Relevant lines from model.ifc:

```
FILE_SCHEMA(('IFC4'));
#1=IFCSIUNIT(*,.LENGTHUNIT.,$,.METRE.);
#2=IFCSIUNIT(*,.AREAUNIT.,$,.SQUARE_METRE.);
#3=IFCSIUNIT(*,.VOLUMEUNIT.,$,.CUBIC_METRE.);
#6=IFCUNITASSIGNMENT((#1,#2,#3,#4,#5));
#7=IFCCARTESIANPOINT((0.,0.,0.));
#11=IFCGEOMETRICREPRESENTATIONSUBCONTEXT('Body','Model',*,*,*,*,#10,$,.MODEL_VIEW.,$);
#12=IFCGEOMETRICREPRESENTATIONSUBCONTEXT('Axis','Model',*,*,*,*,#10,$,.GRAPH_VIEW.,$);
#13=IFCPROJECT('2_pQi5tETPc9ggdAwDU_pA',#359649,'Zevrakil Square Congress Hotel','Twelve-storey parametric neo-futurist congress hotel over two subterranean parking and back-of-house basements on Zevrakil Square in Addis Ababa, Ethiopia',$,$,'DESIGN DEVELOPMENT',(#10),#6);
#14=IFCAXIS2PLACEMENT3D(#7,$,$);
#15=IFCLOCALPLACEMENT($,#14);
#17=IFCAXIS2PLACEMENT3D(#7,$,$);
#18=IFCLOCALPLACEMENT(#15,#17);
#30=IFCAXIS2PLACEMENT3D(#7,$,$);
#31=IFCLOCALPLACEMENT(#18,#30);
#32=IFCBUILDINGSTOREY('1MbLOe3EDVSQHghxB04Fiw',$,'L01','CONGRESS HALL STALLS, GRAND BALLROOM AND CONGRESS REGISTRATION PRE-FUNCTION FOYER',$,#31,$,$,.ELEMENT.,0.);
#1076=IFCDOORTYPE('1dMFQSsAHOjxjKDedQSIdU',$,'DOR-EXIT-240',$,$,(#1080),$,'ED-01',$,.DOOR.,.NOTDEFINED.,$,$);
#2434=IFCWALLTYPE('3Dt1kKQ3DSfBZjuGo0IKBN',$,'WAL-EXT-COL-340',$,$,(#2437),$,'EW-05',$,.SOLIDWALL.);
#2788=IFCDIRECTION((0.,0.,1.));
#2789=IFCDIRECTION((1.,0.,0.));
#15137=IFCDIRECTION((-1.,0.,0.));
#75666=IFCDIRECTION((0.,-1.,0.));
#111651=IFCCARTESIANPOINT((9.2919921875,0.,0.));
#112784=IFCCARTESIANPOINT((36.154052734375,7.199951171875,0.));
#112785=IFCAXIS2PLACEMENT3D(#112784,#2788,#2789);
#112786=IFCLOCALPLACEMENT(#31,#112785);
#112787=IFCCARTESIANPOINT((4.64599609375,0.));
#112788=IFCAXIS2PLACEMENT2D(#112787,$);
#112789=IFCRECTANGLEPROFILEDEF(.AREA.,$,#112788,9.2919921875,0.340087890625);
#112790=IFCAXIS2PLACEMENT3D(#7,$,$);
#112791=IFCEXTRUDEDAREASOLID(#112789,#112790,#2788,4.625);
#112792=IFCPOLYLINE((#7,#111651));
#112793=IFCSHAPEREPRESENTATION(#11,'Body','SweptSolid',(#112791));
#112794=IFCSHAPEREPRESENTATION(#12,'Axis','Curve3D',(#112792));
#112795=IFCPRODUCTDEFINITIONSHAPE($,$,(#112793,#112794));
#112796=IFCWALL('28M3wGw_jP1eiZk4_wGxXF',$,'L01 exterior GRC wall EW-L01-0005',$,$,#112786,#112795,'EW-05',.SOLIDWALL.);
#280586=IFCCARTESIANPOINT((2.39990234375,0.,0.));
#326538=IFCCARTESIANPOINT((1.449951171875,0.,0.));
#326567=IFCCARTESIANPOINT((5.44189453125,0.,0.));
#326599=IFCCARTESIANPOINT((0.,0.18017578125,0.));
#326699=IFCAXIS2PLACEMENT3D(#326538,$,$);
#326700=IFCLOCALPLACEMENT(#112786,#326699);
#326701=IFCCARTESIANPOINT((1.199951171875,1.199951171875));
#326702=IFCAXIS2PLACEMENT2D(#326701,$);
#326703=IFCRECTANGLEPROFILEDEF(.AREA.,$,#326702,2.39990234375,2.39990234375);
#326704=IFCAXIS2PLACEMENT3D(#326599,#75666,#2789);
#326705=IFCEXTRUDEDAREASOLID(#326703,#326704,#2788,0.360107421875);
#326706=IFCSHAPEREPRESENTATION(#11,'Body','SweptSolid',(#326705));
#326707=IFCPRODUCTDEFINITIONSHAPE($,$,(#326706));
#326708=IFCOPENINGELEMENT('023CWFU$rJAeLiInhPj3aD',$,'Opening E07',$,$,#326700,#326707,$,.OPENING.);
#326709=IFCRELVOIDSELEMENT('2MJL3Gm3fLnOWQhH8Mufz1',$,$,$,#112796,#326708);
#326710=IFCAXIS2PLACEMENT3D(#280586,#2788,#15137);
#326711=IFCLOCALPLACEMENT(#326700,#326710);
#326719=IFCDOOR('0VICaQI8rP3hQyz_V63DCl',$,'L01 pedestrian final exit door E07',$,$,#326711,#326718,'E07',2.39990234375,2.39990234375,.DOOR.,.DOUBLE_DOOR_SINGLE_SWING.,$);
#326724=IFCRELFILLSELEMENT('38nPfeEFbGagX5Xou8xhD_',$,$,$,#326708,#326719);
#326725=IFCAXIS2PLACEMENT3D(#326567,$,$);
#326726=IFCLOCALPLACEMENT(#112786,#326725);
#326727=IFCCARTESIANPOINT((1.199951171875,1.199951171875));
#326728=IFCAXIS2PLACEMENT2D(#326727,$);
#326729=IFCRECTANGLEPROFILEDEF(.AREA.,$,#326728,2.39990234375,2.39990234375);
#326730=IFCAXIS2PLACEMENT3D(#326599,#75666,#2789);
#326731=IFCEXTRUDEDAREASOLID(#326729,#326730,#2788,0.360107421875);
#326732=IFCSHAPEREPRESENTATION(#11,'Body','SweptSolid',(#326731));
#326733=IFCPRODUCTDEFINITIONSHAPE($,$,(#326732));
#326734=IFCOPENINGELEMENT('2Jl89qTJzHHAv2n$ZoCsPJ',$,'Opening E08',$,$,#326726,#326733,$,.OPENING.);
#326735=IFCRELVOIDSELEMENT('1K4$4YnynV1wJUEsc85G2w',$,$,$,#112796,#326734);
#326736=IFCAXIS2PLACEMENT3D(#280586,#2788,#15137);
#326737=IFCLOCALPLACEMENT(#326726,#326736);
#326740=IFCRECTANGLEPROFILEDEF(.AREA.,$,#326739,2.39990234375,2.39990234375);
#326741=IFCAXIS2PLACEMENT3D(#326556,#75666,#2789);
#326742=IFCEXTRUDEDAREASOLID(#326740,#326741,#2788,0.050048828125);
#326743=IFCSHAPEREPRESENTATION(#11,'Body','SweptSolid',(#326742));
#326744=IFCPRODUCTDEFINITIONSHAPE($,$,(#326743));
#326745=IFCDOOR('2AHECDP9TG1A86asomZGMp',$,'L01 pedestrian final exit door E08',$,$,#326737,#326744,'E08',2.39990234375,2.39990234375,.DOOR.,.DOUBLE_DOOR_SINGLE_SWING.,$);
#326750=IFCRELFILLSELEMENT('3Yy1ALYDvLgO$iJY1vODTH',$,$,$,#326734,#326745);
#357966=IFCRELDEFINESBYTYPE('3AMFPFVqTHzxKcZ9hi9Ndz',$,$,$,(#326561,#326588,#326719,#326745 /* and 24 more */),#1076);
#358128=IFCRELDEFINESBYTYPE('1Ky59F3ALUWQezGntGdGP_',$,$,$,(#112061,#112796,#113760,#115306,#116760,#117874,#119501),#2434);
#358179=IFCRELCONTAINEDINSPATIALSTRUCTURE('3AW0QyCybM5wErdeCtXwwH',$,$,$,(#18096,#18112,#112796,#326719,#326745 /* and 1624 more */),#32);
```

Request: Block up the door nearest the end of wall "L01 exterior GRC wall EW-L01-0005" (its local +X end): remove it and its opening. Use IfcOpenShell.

```python
import ifcopenshell
import ifcopenshell.api.feature
import ifcopenshell.api.root
import ifcopenshell.geom
import ifcopenshell.util.shape

model = ifcopenshell.open("model.ifc")
settings = ifcopenshell.geom.settings()


def volume(element):
    """Net volume in cubic metres, openings subtracted."""
    shape = ifcopenshell.geom.create_shape(settings, element)
    return ifcopenshell.util.shape.get_volume(shape.geometry)


door = model.by_guid("2AHECDP9TG1A86asomZGMp")
opening = door.FillsVoids[0].RelatingOpeningElement
wall = opening.VoidsElements[0].RelatingBuildingElement
before = volume(wall)

ifcopenshell.api.root.remove_product(model, product=door)
ifcopenshell.api.feature.remove_feature(model, feature=opening)

after = volume(wall)

print(f"wall volume {before:.3f} -> {after:.3f} m3")

model.write("model-out.ifc")
```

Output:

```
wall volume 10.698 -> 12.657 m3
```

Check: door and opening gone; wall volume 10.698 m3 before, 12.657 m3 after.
